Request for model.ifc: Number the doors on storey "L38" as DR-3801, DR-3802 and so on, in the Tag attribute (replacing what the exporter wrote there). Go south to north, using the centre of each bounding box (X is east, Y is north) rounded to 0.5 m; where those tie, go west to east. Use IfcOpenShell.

First a look at what the model holds.

```python
import ifcopenshell
import ifcopenshell.util.element
import ifcopenshell.util.placement

model = ifcopenshell.open("model.ifc")
print(model.schema)
storey = next(s for s in model.by_type("IfcBuildingStorey") if s.Name == "L38")
doors = [e for e in ifcopenshell.util.element.get_decomposition(storey) if e.is_a("IfcDoor")]
for e in sorted(doors, key=lambda e: e.id()):
    origin = ifcopenshell.util.placement.get_local_placement(e.ObjectPlacement)[:3, 3]
    print(e.id(), e.Tag, e.Name, origin.round(2) + 0.0, sep=" | ")
```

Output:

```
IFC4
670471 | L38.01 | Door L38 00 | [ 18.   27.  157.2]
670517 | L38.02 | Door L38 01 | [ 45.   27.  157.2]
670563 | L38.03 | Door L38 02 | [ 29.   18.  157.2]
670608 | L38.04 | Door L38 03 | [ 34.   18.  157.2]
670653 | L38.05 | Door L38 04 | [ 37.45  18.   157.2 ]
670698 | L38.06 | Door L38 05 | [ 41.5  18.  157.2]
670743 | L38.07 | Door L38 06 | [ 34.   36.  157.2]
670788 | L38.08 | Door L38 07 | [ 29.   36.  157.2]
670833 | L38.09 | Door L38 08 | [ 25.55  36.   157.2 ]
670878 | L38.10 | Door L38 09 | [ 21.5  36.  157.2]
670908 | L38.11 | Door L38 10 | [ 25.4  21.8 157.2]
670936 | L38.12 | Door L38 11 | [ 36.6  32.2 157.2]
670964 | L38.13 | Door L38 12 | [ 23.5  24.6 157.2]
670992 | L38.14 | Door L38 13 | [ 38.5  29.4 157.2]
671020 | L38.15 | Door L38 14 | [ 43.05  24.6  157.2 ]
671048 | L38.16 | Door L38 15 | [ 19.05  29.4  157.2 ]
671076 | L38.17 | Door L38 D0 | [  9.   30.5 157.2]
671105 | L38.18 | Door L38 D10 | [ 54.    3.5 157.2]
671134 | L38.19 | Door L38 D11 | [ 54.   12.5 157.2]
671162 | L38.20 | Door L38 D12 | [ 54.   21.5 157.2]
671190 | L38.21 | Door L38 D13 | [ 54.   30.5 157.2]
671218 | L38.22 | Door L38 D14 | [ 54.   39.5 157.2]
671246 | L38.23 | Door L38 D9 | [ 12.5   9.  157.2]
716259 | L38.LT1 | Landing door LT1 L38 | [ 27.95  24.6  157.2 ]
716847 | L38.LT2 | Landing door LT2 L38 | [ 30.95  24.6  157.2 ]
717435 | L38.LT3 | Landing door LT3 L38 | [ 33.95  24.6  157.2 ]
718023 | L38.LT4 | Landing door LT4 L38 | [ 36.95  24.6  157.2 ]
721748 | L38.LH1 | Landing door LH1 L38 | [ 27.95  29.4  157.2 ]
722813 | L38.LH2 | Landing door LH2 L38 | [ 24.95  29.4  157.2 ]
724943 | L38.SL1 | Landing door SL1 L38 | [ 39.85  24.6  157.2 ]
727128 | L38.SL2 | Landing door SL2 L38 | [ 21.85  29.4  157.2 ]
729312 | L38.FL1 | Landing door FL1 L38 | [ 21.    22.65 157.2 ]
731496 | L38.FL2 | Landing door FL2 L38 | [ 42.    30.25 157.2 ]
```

```python
import ifcopenshell
import ifcopenshell.geom
import ifcopenshell.util.element
import ifcopenshell.util.shape

model = ifcopenshell.open("model.ifc")
settings = ifcopenshell.geom.settings()
settings.set("use-world-coords", True)


def centre(element):
    shape = ifcopenshell.geom.create_shape(settings, element)
    return ifcopenshell.util.shape.get_bbox_centroid(shape.geometry)


storey = next(s for s in model.by_type("IfcBuildingStorey") if s.Name == "L38")
doors = [e for e in ifcopenshell.util.element.get_decomposition(storey) if e.is_a("IfcDoor")]

# Insertion points can sit at a corner or the storey origin, so sort by the geometry (in metres).
centres = {e: centre(e) for e in doors}
doors.sort(key=lambda e: (round(centres[e][1] / 0.5), centres[e][0]))

for i, e in enumerate(doors, start=1):
    number = f"DR-38{i:02d}"
    e.Tag = number
    print(e.id(), number)

model.write("model-out.ifc")
```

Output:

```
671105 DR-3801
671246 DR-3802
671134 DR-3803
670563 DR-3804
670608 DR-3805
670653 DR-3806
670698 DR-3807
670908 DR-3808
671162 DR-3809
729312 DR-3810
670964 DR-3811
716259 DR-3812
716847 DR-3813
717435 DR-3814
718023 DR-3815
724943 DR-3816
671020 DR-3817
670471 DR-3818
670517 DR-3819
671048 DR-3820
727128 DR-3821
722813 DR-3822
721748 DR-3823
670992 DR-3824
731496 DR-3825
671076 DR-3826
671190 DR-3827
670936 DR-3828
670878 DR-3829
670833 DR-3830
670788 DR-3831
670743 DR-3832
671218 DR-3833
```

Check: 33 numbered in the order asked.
